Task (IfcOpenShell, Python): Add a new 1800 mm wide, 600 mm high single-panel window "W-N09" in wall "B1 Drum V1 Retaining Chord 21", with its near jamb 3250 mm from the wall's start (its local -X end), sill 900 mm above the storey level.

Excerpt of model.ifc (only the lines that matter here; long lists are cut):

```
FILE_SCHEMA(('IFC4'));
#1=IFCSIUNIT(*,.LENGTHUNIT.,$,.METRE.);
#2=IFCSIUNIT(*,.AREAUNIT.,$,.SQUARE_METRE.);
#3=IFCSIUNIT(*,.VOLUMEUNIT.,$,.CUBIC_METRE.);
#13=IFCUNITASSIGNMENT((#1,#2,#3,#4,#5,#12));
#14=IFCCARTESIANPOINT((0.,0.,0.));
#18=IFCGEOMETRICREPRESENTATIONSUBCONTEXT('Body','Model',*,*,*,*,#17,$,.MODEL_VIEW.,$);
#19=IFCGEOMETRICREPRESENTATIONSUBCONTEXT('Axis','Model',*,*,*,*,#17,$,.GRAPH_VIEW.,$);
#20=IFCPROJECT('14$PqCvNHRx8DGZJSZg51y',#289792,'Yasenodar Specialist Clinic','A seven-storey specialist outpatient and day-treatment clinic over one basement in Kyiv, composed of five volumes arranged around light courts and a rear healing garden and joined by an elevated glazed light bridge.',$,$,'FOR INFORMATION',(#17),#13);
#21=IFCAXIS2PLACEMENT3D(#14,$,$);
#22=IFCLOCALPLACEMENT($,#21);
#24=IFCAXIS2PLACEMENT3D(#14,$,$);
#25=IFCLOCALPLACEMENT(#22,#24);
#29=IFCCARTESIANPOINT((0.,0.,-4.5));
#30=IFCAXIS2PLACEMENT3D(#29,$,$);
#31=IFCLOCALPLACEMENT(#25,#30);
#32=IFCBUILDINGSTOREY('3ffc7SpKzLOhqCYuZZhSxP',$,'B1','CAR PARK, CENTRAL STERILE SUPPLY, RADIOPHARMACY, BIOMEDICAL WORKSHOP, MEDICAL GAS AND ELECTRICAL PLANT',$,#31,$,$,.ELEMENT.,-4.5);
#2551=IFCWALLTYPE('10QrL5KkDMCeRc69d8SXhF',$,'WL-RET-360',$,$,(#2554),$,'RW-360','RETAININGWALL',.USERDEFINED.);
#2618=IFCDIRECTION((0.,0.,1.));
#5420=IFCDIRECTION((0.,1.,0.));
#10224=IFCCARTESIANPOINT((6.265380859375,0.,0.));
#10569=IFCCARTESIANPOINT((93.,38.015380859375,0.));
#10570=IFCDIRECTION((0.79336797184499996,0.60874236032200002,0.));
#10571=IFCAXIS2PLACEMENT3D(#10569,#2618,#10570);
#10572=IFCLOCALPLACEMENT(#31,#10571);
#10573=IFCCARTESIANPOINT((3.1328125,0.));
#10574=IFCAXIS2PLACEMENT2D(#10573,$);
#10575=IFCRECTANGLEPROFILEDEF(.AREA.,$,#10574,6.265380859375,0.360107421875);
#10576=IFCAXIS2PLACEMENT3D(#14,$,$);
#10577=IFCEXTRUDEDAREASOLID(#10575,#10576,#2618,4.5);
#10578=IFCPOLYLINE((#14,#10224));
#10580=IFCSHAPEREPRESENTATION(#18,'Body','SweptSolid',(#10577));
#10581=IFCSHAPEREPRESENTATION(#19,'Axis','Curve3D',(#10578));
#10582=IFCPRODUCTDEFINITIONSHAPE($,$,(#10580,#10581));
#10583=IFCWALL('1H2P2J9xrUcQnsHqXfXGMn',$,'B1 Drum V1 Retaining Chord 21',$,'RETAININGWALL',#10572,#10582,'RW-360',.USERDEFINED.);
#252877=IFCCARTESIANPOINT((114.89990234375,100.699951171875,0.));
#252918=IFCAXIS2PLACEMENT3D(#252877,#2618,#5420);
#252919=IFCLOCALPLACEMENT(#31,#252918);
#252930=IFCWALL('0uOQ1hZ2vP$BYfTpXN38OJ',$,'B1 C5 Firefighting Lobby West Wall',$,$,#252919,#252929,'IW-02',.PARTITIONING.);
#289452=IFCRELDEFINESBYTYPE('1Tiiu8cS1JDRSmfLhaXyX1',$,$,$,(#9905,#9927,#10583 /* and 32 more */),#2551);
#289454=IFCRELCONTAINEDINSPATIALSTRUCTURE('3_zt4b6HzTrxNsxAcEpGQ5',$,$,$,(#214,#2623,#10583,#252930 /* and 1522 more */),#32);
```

```python
import numpy as np
import ifcopenshell
import ifcopenshell.api.feature
import ifcopenshell.api.geometry
import ifcopenshell.api.root
import ifcopenshell.api.spatial
import ifcopenshell.geom
import ifcopenshell.util.element
import ifcopenshell.util.placement
import ifcopenshell.util.representation
import ifcopenshell.util.shape
import ifcopenshell.util.unit

model = ifcopenshell.open("model.ifc")
unit_scale = ifcopenshell.util.unit.calculate_unit_scale(model)
settings = ifcopenshell.geom.settings()


def volume(element):
    """Net volume in cubic metres, openings subtracted."""
    shape = ifcopenshell.geom.create_shape(settings, element)
    return ifcopenshell.util.shape.get_volume(shape.geometry)


wall = model.by_guid("1H2P2J9xrUcQnsHqXfXGMn")
storey = ifcopenshell.util.element.get_container(wall, ifc_class="IfcBuildingStorey")
context = ifcopenshell.util.representation.get_context(model, "Model", "Body", "MODEL_VIEW")
before = volume(wall)

width, height, from_end, sill = 1.8, 0.6, 3.25, 0.9  # metres

# The wall runs along its own X axis, and the end named is its -X end.
wall_shape = ifcopenshell.geom.create_shape(settings, wall)
x, y, z = ifcopenshell.util.shape.get_vertices(wall_shape.geometry).T
start = x.min() + from_end
face, thickness = float(y.min()), float(y.max() - y.min())
wall_matrix = ifcopenshell.util.placement.get_local_placement(wall.ObjectPlacement)
level = ifcopenshell.util.placement.get_local_placement(storey.ObjectPlacement)[2, 3]


def in_wall(x, y):
    """Placement at x, y metres in the wall's axes, at sill height."""
    matrix = wall_matrix.copy()
    matrix[:, 3] = wall_matrix @ np.array([x / unit_scale, y / unit_scale, 0.0, 1.0])
    matrix[2, 3] = level + sill / unit_scale
    return matrix


# Opening: a box that overshoots both wall faces by 50 mm.
opening = ifcopenshell.api.root.create_entity(model, ifc_class="IfcOpeningElement", predefined_type="OPENING")
box = ifcopenshell.api.geometry.add_wall_representation(
    model, context=context, length=width, height=height, thickness=thickness + 0.1
)
ifcopenshell.api.geometry.assign_representation(model, product=opening, representation=box)
ifcopenshell.api.geometry.edit_object_placement(model, product=opening, matrix=in_wall(start, face - 0.05), is_si=False)
ifcopenshell.api.feature.add_feature(model, feature=opening, element=wall)

window = ifcopenshell.api.root.create_entity(model, ifc_class="IfcWindow", name="W-N09", predefined_type="WINDOW")
window.OverallWidth, window.OverallHeight = width / unit_scale, height / unit_scale
window.PartitioningType = "SINGLE_PANEL"
body = ifcopenshell.api.geometry.add_window_representation(
    model,
    context=context,
    overall_width=window.OverallWidth,
    overall_height=window.OverallHeight,
    partition_type="SINGLE_PANEL",
)
ifcopenshell.api.geometry.assign_representation(model, product=window, representation=body)
ifcopenshell.api.spatial.assign_container(model, products=[window], relating_structure=storey)
ifcopenshell.api.feature.add_filling(model, opening=opening, element=window)

# Centre the window in the wall's thickness.
ifcopenshell.api.geometry.edit_object_placement(model, product=window, matrix=in_wall(start, face), is_si=False)
window_shape = ifcopenshell.geom.create_shape(settings, window)
depth = ifcopenshell.util.shape.get_vertices(window_shape.geometry)[:, 1]
offset = face + thickness / 2 - (depth.min() + depth.max()) / 2
ifcopenshell.api.geometry.edit_object_placement(model, product=window, matrix=in_wall(start, offset), is_si=False)

after = volume(wall)

print(f"wall volume {before:.3f} -> {after:.3f} m3")

model.write("model_v2.ifc")
```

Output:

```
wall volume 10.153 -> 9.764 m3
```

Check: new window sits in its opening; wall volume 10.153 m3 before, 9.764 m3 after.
